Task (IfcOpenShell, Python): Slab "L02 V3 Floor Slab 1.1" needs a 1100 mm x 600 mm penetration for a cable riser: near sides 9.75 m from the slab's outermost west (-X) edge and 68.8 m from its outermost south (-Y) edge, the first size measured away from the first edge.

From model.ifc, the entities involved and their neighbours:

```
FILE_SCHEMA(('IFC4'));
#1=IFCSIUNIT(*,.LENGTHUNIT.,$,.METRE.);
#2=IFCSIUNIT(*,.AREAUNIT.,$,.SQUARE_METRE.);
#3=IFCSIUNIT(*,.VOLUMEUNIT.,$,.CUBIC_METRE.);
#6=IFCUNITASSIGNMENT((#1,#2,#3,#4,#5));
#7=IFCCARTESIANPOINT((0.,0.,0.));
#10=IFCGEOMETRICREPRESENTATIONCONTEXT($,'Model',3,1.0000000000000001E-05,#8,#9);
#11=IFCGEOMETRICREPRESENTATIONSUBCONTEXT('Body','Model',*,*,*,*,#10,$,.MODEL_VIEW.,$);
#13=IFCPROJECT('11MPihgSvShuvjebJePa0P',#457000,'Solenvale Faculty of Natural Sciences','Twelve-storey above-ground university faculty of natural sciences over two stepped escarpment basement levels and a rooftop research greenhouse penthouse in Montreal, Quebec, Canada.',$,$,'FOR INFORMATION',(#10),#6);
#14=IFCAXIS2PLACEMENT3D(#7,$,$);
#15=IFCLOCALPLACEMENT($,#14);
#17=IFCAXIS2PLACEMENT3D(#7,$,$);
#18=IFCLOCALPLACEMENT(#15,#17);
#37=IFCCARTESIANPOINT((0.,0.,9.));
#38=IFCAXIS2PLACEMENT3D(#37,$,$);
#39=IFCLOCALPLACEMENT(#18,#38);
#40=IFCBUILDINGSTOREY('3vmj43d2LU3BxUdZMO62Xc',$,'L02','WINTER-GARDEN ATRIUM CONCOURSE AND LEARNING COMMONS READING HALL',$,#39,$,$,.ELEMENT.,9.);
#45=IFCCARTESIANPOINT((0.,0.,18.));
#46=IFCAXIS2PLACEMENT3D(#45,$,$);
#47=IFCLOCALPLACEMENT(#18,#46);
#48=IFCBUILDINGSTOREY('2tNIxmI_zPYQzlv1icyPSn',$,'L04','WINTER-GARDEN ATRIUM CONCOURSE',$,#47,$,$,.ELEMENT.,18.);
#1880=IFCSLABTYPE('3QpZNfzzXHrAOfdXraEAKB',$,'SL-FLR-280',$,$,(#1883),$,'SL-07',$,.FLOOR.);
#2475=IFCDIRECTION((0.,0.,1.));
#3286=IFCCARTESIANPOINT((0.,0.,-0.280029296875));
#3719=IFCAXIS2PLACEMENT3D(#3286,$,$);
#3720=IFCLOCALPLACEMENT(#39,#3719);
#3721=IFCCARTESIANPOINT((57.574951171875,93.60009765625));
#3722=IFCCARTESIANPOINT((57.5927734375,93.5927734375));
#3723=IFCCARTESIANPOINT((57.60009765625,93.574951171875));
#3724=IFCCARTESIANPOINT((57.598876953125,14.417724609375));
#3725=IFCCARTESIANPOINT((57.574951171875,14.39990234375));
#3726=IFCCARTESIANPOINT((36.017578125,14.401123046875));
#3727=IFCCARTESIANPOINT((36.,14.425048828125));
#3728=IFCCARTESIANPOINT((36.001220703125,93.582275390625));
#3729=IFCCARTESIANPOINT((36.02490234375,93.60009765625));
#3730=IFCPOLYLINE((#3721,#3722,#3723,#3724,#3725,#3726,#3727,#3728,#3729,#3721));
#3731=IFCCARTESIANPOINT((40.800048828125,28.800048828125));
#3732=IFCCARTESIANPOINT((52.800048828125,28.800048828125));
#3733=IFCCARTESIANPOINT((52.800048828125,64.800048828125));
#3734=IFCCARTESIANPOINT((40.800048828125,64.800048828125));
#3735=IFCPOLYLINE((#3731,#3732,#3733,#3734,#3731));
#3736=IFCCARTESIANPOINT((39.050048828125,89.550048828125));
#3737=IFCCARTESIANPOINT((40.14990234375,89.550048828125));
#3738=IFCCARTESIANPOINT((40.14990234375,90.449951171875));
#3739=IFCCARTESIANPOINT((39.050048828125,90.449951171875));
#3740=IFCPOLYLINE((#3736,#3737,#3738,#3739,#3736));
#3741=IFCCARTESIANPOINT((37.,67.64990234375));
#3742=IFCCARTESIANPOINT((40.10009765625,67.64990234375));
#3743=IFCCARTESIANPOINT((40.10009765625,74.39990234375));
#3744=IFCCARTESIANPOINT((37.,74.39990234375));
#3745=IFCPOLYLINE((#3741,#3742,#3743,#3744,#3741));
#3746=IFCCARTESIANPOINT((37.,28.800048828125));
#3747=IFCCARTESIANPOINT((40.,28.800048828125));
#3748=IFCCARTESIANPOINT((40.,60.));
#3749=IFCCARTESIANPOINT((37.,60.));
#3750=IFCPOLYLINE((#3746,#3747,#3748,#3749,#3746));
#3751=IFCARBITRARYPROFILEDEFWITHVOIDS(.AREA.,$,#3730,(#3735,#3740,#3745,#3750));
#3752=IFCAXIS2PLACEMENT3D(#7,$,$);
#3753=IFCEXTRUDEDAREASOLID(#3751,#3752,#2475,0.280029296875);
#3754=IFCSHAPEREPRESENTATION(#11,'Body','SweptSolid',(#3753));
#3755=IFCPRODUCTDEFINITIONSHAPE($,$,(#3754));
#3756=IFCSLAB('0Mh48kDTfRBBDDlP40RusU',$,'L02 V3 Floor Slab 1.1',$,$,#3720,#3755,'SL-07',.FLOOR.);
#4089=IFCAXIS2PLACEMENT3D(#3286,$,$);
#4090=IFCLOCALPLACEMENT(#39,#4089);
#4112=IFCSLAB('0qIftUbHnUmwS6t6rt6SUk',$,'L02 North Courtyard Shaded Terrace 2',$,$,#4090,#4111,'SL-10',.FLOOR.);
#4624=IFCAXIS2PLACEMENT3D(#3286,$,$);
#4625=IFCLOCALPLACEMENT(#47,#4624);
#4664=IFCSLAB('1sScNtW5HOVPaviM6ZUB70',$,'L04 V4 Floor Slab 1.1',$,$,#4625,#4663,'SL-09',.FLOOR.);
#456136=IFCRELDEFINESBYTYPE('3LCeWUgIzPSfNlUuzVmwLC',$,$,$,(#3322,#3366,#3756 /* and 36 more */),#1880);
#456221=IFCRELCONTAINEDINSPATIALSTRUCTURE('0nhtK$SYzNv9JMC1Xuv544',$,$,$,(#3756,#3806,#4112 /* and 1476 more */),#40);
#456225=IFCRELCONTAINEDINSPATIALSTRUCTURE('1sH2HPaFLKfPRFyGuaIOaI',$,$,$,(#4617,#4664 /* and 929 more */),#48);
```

```python
import numpy as np
import ifcopenshell
import ifcopenshell.api.feature
import ifcopenshell.api.geometry
import ifcopenshell.api.root
import ifcopenshell.geom
import ifcopenshell.util.placement
import ifcopenshell.util.representation
import ifcopenshell.util.shape
import ifcopenshell.util.unit

model = ifcopenshell.open("model.ifc")
unit_scale = ifcopenshell.util.unit.calculate_unit_scale(model)
settings = ifcopenshell.geom.settings()


def volume(element):
    """Net volume in cubic metres, openings subtracted."""
    shape = ifcopenshell.geom.create_shape(settings, element)
    return ifcopenshell.util.shape.get_volume(shape.geometry)


slab = model.by_guid("0Mh48kDTfRBBDDlP40RusU")
before = volume(slab)

# Extent in the slab's own axes, in metres. The edges named are its -X and -Y sides.
slab_shape = ifcopenshell.geom.create_shape(settings, slab)
vertices = ifcopenshell.util.shape.get_vertices(slab_shape.geometry)
x_min, y_min, bottom = vertices.min(axis=0)
top = vertices[:, 2].max()

opening = ifcopenshell.api.root.create_entity(model, ifc_class="IfcOpeningElement", name="Cable riser opening", predefined_type="OPENING")
context = ifcopenshell.util.representation.get_context(model, "Model", "Body", "MODEL_VIEW")
width, depth = 1.1, 0.6
outline = [(0.0, 0.0), (width, 0.0), (width, depth), (0.0, depth), (0.0, 0.0)]
# Overshoot both faces by 50 mm so the cut is clean.
shape = ifcopenshell.api.geometry.add_slab_representation(
    model, context=context, depth=top - bottom + 0.1, polyline=outline
)
ifcopenshell.api.geometry.assign_representation(model, product=opening, representation=shape)

matrix = ifcopenshell.util.placement.get_local_placement(slab.ObjectPlacement)
matrix[:, 3] = matrix @ np.append(np.array([x_min + 9.75, y_min + 68.8, bottom - 0.05]) / unit_scale, 1.0)
ifcopenshell.api.geometry.edit_object_placement(model, product=opening, matrix=matrix, is_si=False)
ifcopenshell.api.feature.add_feature(model, feature=opening, element=slab)

after = volume(slab)

print(f"slab volume {before:.3f} -> {after:.3f} m3")

model.write("model-out.ifc")
```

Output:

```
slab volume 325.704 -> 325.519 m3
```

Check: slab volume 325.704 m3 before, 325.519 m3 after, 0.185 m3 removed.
